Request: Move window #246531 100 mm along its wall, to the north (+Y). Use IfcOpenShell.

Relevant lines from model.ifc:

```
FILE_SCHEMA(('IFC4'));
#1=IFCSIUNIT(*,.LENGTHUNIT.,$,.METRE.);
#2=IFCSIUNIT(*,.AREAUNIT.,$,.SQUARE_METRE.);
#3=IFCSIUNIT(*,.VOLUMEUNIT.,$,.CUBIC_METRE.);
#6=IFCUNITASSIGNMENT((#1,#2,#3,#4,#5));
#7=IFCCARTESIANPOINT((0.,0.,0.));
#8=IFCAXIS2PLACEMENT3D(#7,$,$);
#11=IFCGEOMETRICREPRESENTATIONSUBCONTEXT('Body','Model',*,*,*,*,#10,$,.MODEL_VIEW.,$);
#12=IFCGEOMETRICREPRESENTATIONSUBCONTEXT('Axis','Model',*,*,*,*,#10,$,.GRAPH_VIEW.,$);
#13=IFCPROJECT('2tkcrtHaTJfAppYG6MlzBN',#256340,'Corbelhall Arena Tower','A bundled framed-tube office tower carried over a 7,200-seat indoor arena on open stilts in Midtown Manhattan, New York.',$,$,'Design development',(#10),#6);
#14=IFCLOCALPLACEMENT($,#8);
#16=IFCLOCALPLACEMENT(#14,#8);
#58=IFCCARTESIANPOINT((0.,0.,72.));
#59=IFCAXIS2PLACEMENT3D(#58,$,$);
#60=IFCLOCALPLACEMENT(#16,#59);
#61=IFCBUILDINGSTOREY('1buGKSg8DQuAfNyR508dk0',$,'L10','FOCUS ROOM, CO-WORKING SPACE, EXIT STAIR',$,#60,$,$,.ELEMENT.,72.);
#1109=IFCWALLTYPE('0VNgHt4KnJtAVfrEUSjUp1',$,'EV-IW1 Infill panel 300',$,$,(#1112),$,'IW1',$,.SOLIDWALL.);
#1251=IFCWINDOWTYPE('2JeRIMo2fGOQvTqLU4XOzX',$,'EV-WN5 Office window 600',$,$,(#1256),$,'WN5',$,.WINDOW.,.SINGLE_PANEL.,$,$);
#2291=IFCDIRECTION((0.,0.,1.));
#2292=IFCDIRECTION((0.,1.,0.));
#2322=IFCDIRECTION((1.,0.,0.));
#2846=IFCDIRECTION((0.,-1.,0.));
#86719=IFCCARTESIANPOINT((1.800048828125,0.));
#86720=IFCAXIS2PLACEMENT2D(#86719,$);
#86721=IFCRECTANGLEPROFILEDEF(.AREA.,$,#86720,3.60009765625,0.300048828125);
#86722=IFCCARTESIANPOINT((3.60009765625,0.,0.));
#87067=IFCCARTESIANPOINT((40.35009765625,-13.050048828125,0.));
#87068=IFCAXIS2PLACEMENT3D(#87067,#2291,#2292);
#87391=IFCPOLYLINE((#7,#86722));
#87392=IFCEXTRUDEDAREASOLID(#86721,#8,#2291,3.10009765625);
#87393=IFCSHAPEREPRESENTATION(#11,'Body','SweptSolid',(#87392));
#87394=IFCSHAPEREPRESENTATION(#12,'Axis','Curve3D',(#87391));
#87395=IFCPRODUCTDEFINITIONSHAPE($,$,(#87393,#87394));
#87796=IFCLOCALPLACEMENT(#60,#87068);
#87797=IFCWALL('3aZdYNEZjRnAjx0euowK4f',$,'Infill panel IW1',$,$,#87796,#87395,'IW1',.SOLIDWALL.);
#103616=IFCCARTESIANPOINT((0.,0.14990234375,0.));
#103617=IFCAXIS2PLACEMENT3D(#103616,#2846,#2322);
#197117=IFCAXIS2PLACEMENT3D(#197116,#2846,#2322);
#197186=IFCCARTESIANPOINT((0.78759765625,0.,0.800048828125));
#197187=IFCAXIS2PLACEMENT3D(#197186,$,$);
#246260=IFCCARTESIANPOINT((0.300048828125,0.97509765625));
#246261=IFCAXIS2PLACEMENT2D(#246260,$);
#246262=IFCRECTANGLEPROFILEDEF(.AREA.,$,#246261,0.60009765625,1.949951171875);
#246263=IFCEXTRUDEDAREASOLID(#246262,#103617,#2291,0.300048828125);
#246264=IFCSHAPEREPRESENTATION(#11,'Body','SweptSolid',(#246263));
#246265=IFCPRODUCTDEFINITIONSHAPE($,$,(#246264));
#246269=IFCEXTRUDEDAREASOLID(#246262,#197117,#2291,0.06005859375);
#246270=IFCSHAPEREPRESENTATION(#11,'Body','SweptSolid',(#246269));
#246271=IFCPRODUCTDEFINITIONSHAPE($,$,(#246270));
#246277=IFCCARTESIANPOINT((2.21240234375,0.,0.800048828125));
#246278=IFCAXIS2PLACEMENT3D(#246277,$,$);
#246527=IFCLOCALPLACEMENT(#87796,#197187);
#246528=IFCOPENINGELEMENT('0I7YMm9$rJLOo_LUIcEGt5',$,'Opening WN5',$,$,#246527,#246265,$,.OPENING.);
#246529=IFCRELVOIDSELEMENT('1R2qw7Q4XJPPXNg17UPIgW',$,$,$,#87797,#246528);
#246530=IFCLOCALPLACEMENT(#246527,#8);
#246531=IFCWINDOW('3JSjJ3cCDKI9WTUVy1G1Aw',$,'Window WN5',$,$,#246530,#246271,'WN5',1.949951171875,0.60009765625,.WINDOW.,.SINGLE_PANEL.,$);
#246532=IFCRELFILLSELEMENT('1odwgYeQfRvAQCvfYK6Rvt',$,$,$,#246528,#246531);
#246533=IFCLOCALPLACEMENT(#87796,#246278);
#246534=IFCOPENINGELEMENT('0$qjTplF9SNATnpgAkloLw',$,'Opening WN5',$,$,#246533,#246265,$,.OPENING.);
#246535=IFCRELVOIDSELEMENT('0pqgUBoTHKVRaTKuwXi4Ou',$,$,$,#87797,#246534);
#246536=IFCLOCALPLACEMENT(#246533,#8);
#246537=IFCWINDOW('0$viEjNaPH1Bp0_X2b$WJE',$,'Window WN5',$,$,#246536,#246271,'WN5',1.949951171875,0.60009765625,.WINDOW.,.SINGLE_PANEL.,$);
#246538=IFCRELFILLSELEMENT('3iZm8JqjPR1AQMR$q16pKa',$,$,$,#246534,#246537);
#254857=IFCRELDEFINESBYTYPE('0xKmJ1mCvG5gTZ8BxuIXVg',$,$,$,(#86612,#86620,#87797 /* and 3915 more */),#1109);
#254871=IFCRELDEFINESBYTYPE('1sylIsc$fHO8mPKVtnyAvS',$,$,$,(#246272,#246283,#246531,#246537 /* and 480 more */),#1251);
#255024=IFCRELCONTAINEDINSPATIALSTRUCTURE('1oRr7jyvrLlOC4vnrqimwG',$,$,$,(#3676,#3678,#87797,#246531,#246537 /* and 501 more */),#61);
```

```python
import ifcopenshell
import ifcopenshell.api.geometry
import ifcopenshell.util.placement
import ifcopenshell.util.unit

model = ifcopenshell.open("model.ifc")
unit_scale = ifcopenshell.util.unit.calculate_unit_scale(model)

window = model.by_guid("3JSjJ3cCDKI9WTUVy1G1Aw")
opening = window.FillsVoids[0].RelatingOpeningElement
wall = opening.VoidsElements[0].RelatingBuildingElement

wall_matrix = ifcopenshell.util.placement.get_local_placement(wall.ObjectPlacement)
shift = wall_matrix[:3, 0] * 0.1 / unit_scale
before = ifcopenshell.util.placement.get_local_placement(window.ObjectPlacement)[:3, 3].copy()

# The window is placed relative to its opening, so it follows when the opening moves.
matrix = ifcopenshell.util.placement.get_local_placement(opening.ObjectPlacement)
matrix[:3, 3] += shift
ifcopenshell.api.geometry.edit_object_placement(
    model, product=opening, matrix=matrix, is_si=False, should_transform_children=True
)

after = ifcopenshell.util.placement.get_local_placement(window.ObjectPlacement)[:3, 3]
print("window moved by", (after - before).round(3) + 0.0)

model.write("model_rev.ifc")
```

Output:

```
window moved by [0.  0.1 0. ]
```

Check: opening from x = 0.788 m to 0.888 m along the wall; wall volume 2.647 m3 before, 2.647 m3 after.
